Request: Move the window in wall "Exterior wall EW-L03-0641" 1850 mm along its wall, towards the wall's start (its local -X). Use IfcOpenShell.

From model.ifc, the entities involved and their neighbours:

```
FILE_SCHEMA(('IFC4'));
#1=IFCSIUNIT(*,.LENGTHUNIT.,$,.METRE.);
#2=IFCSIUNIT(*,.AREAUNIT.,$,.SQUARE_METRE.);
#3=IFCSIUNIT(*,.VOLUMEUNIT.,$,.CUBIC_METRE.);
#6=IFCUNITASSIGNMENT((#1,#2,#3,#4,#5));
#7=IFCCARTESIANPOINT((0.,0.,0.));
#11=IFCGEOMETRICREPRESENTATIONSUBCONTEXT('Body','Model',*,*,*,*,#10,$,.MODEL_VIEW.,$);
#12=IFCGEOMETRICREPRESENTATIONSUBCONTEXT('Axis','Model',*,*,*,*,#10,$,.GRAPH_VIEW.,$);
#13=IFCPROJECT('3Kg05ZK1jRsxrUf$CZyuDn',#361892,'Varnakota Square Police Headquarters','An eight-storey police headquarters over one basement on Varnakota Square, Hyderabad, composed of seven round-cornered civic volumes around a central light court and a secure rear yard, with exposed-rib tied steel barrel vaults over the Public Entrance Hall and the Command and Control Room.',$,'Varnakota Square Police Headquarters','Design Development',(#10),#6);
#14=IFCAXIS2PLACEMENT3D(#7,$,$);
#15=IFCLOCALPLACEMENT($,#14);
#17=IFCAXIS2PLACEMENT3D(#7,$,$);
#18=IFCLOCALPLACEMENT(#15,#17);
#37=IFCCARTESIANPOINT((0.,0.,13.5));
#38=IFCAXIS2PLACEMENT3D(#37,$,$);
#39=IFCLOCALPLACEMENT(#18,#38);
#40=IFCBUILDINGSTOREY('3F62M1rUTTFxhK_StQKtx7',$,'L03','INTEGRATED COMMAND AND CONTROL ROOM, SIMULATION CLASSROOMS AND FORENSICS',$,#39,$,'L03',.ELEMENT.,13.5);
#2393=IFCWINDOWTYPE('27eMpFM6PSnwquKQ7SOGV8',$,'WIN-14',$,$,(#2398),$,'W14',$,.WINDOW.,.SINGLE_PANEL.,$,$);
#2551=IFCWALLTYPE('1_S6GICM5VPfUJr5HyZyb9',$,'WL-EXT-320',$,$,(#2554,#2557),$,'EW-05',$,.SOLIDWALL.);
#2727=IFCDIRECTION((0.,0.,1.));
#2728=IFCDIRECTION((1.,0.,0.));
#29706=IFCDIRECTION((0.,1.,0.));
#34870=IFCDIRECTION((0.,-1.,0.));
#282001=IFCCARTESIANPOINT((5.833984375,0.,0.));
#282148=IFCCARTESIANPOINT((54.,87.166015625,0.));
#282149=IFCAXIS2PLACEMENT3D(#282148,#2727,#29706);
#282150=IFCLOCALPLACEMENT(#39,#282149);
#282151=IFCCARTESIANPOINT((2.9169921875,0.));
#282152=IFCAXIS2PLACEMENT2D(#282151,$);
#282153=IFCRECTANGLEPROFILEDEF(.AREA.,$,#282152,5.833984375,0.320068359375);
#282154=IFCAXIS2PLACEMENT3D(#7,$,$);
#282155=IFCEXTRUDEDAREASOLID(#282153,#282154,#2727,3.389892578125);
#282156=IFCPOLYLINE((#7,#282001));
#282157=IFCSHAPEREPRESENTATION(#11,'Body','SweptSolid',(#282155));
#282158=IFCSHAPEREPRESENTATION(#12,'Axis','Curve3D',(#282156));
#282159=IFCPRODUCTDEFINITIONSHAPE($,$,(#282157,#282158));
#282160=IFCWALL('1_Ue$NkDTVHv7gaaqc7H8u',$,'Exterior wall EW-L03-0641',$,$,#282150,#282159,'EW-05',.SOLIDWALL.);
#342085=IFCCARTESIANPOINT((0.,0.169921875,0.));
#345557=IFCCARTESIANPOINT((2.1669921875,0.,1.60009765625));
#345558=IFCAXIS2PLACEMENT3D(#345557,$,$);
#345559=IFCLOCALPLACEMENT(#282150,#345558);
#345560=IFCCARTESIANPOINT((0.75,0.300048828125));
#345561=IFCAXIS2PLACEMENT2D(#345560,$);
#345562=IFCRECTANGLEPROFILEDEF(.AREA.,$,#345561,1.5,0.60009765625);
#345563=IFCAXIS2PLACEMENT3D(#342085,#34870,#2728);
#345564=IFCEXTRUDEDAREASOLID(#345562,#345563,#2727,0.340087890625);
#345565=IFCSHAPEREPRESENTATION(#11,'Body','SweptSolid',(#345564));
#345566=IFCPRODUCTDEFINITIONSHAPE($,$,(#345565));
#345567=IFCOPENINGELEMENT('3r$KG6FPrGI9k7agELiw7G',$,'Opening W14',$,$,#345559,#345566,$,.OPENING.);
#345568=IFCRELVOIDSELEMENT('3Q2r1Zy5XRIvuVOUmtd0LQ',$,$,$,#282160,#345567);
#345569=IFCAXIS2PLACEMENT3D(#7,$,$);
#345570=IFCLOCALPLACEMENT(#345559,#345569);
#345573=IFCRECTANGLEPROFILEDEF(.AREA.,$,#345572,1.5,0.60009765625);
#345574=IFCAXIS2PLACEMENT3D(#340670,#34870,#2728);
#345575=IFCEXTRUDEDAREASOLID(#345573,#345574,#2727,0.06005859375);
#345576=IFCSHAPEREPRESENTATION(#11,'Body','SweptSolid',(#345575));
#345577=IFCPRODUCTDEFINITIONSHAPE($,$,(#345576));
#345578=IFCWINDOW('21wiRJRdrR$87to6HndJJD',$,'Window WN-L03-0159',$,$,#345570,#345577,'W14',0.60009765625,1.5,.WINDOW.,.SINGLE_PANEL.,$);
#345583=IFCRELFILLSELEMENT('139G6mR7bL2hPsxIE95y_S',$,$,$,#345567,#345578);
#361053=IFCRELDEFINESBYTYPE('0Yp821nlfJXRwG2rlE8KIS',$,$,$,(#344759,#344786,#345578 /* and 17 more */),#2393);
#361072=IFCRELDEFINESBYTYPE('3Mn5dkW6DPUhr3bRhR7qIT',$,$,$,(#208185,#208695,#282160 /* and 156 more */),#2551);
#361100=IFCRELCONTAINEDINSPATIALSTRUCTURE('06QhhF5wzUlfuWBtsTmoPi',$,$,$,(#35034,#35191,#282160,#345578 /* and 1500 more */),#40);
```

```python
import ifcopenshell
import ifcopenshell.api.geometry
import ifcopenshell.util.placement
import ifcopenshell.util.unit

model = ifcopenshell.open("model.ifc")
unit_scale = ifcopenshell.util.unit.calculate_unit_scale(model)

window = model.by_guid("21wiRJRdrR$87to6HndJJD")
opening = window.FillsVoids[0].RelatingOpeningElement
wall = opening.VoidsElements[0].RelatingBuildingElement

wall_matrix = ifcopenshell.util.placement.get_local_placement(wall.ObjectPlacement)
shift = wall_matrix[:3, 0] * -1.85 / unit_scale
before = ifcopenshell.util.placement.get_local_placement(window.ObjectPlacement)[:3, 3].copy()

# The window is placed relative to its opening, so it follows when the opening moves.
matrix = ifcopenshell.util.placement.get_local_placement(opening.ObjectPlacement)
matrix[:3, 3] += shift
ifcopenshell.api.geometry.edit_object_placement(
    model, product=opening, matrix=matrix, is_si=False, should_transform_children=True
)

after = ifcopenshell.util.placement.get_local_placement(window.ObjectPlacement)[:3, 3]
print("window moved by", (after - before).round(3) + 0.0)

model.write("model_v2.ifc")
```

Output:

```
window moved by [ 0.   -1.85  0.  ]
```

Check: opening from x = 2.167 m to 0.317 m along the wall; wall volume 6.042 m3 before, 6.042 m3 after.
